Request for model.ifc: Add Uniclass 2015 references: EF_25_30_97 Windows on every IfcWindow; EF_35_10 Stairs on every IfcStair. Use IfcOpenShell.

First a look at what the model holds.

```python
import ifcopenshell

model = ifcopenshell.open("model.ifc")
print(model.schema)
print("classifications:", [c.Name for c in model.by_type("IfcClassification")])
for ifc_class in ("IfcDoor", "IfcRoof", "IfcStair", "IfcWall", "IfcWindow"):
    print(ifc_class, len(model.by_type(ifc_class)))
```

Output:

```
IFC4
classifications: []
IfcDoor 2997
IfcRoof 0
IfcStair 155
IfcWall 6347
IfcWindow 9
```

```python
import ifcopenshell
import ifcopenshell.api.classification

model = ifcopenshell.open("model.ifc")

system = ifcopenshell.api.classification.add_classification(model, classification="Uniclass 2015")

codes = {
    "IfcWindow": ("EF_25_30_97", "Windows"),
    "IfcStair": ("EF_35_10", "Stairs"),
}
for ifc_class, (code, name) in codes.items():
    products = model.by_type(ifc_class)
    ifcopenshell.api.classification.add_reference(
        model, products=products, classification=system, identification=code, name=name
    )
    print(code, len(products))

model.write("model_updated.ifc")
```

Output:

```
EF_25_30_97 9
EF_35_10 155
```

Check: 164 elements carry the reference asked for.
